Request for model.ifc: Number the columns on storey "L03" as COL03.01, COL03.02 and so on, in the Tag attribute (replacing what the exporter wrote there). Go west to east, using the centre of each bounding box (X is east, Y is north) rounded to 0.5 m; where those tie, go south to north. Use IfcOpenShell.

First a look at what the model holds.

```python
import ifcopenshell
import ifcopenshell.util.element
import ifcopenshell.util.placement

model = ifcopenshell.open("model.ifc")
print(model.schema)
storey = next(s for s in model.by_type("IfcBuildingStorey") if s.Name == "L03")
columns = [e for e in ifcopenshell.util.element.get_decomposition(storey) if e.is_a("IfcColumn")]
for e in sorted(columns, key=lambda e: e.id()):
    origin = ifcopenshell.util.placement.get_local_placement(e.ObjectPlacement)[:3, 3]
    print(e.id(), e.Tag, e.Name, origin.round(2) + 0.0, sep=" | ")
```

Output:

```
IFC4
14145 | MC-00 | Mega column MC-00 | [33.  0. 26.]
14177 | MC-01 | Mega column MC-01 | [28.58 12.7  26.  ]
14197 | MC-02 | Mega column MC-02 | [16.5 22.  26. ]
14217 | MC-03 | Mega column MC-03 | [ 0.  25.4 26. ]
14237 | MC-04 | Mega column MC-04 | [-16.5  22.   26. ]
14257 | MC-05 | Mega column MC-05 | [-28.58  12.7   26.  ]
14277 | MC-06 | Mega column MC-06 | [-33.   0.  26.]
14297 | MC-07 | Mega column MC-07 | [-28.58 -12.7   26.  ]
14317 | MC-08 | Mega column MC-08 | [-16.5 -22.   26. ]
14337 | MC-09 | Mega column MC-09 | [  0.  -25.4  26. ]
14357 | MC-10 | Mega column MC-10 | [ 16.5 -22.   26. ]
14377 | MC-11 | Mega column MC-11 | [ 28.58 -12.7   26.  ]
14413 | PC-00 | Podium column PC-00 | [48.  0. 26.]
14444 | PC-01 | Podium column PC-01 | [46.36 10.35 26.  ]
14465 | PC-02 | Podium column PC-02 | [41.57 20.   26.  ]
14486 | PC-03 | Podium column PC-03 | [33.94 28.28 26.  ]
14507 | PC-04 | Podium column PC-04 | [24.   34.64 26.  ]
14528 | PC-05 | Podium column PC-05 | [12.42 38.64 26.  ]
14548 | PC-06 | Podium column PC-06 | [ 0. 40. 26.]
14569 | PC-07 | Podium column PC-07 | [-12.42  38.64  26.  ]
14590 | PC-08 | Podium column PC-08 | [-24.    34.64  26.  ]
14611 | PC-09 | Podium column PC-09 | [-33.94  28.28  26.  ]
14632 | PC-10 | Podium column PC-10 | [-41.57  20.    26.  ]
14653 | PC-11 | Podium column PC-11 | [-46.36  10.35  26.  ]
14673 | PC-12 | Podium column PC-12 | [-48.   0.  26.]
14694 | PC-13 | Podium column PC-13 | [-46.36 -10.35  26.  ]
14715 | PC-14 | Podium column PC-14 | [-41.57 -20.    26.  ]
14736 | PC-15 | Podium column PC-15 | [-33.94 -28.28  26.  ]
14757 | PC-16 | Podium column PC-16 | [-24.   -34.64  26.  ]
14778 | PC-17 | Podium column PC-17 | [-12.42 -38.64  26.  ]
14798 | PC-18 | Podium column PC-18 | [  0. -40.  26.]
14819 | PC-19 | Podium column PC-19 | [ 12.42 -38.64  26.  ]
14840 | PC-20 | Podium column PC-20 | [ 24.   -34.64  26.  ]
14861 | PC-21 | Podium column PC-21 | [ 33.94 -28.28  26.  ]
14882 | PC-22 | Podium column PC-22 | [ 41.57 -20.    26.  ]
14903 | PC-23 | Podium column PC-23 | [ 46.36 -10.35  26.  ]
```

```python
import ifcopenshell
import ifcopenshell.geom
import ifcopenshell.util.element
import ifcopenshell.util.shape

model = ifcopenshell.open("model.ifc")
settings = ifcopenshell.geom.settings()
settings.set("use-world-coords", True)


def centre(element):
    shape = ifcopenshell.geom.create_shape(settings, element)
    return ifcopenshell.util.shape.get_bbox_centroid(shape.geometry)


storey = next(s for s in model.by_type("IfcBuildingStorey") if s.Name == "L03")
columns = [e for e in ifcopenshell.util.element.get_decomposition(storey) if e.is_a("IfcColumn")]

# Insertion points can sit at a corner or the storey origin, so sort by the geometry (in metres).
centres = {e: centre(e) for e in columns}
columns.sort(key=lambda e: (round(centres[e][0] / 0.5), centres[e][1]))

for i, e in enumerate(columns, start=1):
    number = f"COL03.{i:02d}"
    e.Tag = number
    print(e.id(), number)

model.write("model_rev.ifc")
```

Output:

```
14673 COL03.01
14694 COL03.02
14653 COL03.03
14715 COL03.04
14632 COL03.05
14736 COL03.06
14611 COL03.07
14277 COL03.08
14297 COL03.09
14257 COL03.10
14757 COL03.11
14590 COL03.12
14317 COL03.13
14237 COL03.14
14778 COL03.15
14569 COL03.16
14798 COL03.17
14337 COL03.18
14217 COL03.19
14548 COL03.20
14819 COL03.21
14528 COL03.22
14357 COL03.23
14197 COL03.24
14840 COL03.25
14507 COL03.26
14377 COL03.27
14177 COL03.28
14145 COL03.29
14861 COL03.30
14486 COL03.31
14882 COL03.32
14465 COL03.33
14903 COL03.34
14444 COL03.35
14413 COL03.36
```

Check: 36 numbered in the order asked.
